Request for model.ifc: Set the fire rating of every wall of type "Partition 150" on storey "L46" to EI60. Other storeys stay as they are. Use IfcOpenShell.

First a look at what the model holds.

```python
import ifcopenshell
import ifcopenshell.util.element

model = ifcopenshell.open("model.ifc")
print(model.schema)
storey = next(s for s in model.by_type("IfcBuildingStorey") if s.Name == "L46")
walls = [e for e in ifcopenshell.util.element.get_decomposition(storey) if e.is_a("IfcWall")]
seen = {}
for e in walls:
    element_type = ifcopenshell.util.element.get_type(e)
    key = (element_type.Name if element_type != e and element_type else None, ifcopenshell.util.element.get_pset(e, "Pset_WallCommon", "FireRating"))
    seen[key] = seen.get(key, 0) + 1
for (name, value), count in sorted(seen.items(), key=str):
    print(count, "x", name, "|", value)
```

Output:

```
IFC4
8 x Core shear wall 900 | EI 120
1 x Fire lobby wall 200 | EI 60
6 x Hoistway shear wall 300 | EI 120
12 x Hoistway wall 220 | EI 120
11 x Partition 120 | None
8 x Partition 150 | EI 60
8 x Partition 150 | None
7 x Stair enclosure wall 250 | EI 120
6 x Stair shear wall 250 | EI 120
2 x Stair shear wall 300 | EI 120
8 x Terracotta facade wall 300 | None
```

```python
import ifcopenshell
import ifcopenshell.api.pset
import ifcopenshell.util.element

model = ifcopenshell.open("model.ifc")

storey = next(s for s in model.by_type("IfcBuildingStorey") if s.Name == "L46")
walls = [e for e in ifcopenshell.util.element.get_decomposition(storey) if e.is_a("IfcWall")]

count = 0
for e in walls:
    element_type = ifcopenshell.util.element.get_type(e)
    if element_type in (None, e) or element_type.Name != "Partition 150":
        continue
    found = ifcopenshell.util.element.get_pset(e, "Pset_WallCommon", should_inherit=False)
    if found:
        pset = model.by_id(found["id"])
        if len(ifcopenshell.util.element.get_elements_by_pset(pset)) > 1:
            pset = ifcopenshell.api.pset.unshare_pset(model, products=[e], pset=pset)[0]
    else:
        pset = ifcopenshell.api.pset.add_pset(model, product=e, name="Pset_WallCommon")
    ifcopenshell.api.pset.edit_pset(model, pset=pset, properties={"FireRating": "EI60"})
    count += 1

print(count, "walls updated")

model.write("model-out.ifc")
```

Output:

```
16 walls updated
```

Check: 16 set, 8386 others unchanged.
